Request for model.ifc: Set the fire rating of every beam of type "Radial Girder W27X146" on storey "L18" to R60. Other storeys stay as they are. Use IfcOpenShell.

First a look at what the model holds.

```python
import ifcopenshell
import ifcopenshell.util.element

model = ifcopenshell.open("model.ifc")
print(model.schema)
storey = next(s for s in model.by_type("IfcBuildingStorey") if s.Name == "L18")
beams = [e for e in ifcopenshell.util.element.get_decomposition(storey) if e.is_a("IfcBeam")]
seen = {}
for e in beams:
    element_type = ifcopenshell.util.element.get_type(e)
    key = (element_type.Name if element_type != e and element_type else None, ifcopenshell.util.element.get_pset(e, "Pset_BeamCommon", "FireRating"))
    seen[key] = seen.get(key, 0) + 1
for (name, value), count in sorted(seen.items(), key=str):
    print(count, "x", name, "|", value)
```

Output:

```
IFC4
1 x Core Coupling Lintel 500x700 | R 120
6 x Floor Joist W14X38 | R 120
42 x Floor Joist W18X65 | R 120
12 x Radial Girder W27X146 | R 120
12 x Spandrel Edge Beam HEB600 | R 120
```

```python
import ifcopenshell
import ifcopenshell.api.pset
import ifcopenshell.util.element

model = ifcopenshell.open("model.ifc")

storey = next(s for s in model.by_type("IfcBuildingStorey") if s.Name == "L18")
beams = [e for e in ifcopenshell.util.element.get_decomposition(storey) if e.is_a("IfcBeam")]

count = 0
for e in beams:
    element_type = ifcopenshell.util.element.get_type(e)
    if element_type in (None, e) or element_type.Name != "Radial Girder W27X146":
        continue
    found = ifcopenshell.util.element.get_pset(e, "Pset_BeamCommon", should_inherit=False)
    if found:
        pset = model.by_id(found["id"])
        if len(ifcopenshell.util.element.get_elements_by_pset(pset)) > 1:
            pset = ifcopenshell.api.pset.unshare_pset(model, products=[e], pset=pset)[0]
    else:
        pset = ifcopenshell.api.pset.add_pset(model, product=e, name="Pset_BeamCommon")
    ifcopenshell.api.pset.edit_pset(model, pset=pset, properties={"FireRating": "R60"})
    count += 1

print(count, "beams updated")

model.write("model_v2.ifc")
```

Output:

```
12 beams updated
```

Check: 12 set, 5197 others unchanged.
